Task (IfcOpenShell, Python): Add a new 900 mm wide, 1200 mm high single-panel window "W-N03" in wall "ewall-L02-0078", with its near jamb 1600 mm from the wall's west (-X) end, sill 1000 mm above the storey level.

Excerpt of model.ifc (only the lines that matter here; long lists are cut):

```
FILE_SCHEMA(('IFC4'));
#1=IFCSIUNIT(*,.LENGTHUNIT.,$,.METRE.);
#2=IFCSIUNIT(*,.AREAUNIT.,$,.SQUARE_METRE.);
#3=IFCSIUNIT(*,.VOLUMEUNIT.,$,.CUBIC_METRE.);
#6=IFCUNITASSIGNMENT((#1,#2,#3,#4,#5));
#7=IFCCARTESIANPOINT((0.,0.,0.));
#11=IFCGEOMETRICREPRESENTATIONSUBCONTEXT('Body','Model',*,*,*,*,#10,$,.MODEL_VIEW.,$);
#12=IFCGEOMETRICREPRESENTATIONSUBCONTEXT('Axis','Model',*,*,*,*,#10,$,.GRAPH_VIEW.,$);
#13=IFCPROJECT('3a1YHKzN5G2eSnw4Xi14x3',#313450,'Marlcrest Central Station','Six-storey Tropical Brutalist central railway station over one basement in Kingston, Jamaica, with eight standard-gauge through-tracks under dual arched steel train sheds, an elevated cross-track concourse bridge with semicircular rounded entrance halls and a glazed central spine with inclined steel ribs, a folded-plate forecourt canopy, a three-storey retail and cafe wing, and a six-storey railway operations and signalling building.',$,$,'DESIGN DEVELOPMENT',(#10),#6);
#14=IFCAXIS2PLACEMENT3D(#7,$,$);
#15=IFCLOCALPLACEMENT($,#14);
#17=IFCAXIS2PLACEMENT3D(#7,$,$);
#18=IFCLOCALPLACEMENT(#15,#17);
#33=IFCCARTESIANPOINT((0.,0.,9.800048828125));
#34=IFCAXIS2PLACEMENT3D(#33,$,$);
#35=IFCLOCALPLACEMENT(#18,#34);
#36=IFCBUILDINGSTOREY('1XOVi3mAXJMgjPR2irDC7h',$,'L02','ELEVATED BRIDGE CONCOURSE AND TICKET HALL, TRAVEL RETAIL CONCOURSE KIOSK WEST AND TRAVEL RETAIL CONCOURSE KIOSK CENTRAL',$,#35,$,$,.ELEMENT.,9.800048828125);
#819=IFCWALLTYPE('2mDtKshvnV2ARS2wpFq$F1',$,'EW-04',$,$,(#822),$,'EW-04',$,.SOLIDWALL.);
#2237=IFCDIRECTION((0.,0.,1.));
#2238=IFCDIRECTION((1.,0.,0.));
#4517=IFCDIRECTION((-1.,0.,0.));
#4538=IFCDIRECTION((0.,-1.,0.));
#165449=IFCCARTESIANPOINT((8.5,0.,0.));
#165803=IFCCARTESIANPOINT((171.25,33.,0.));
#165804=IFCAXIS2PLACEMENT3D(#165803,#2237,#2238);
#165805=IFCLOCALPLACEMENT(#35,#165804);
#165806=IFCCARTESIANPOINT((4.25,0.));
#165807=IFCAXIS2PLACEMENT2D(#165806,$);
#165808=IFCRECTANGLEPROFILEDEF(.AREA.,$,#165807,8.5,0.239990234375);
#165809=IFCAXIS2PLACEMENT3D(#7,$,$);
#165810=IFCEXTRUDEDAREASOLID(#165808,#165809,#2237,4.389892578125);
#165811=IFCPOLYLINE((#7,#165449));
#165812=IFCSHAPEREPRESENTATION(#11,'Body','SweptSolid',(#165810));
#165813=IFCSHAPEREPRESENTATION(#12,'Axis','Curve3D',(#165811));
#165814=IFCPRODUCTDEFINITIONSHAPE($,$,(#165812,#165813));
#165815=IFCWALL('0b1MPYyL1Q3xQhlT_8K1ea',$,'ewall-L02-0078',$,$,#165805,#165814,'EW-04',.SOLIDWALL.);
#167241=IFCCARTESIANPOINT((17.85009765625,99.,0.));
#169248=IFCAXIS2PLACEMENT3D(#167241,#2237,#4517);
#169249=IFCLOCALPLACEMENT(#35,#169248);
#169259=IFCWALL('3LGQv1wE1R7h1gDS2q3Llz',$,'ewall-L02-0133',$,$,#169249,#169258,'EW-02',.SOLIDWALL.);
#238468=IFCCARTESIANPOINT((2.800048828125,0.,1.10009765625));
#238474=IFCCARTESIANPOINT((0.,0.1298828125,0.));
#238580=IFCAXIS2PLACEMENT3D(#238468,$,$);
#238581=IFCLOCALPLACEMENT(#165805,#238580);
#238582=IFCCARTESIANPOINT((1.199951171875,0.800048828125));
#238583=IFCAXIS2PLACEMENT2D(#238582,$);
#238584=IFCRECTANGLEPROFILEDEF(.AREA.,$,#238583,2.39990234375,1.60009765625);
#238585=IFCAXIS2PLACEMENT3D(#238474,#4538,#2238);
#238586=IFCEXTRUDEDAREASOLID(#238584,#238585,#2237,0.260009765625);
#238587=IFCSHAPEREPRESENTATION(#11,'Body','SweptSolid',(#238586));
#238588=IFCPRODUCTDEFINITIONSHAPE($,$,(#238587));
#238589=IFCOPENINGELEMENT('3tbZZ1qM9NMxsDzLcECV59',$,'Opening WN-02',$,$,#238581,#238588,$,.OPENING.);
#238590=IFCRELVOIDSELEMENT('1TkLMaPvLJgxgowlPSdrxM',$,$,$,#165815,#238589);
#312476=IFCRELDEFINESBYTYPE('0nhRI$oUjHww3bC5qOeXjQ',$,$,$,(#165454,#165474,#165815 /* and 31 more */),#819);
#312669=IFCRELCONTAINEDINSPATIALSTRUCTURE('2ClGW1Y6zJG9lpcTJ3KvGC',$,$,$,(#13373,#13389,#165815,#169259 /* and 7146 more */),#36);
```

```python
import numpy as np
import ifcopenshell
import ifcopenshell.api.feature
import ifcopenshell.api.geometry
import ifcopenshell.api.root
import ifcopenshell.api.spatial
import ifcopenshell.geom
import ifcopenshell.util.element
import ifcopenshell.util.placement
import ifcopenshell.util.representation
import ifcopenshell.util.shape
import ifcopenshell.util.unit

model = ifcopenshell.open("model.ifc")
unit_scale = ifcopenshell.util.unit.calculate_unit_scale(model)
settings = ifcopenshell.geom.settings()


def volume(element):
    """Net volume in cubic metres, openings subtracted."""
    shape = ifcopenshell.geom.create_shape(settings, element)
    return ifcopenshell.util.shape.get_volume(shape.geometry)


wall = model.by_guid("0b1MPYyL1Q3xQhlT_8K1ea")
storey = ifcopenshell.util.element.get_container(wall, ifc_class="IfcBuildingStorey")
context = ifcopenshell.util.representation.get_context(model, "Model", "Body", "MODEL_VIEW")
before = volume(wall)

width, height, from_end, sill = 0.9, 1.2, 1.6, 1  # metres

# The wall runs along its own X axis, and the end named is its -X end.
wall_shape = ifcopenshell.geom.create_shape(settings, wall)
x, y, z = ifcopenshell.util.shape.get_vertices(wall_shape.geometry).T
start = x.min() + from_end
face, thickness = float(y.min()), float(y.max() - y.min())
wall_matrix = ifcopenshell.util.placement.get_local_placement(wall.ObjectPlacement)
level = ifcopenshell.util.placement.get_local_placement(storey.ObjectPlacement)[2, 3]


def in_wall(x, y):
    """Placement at x, y metres in the wall's axes, at sill height."""
    matrix = wall_matrix.copy()
    matrix[:, 3] = wall_matrix @ np.array([x / unit_scale, y / unit_scale, 0.0, 1.0])
    matrix[2, 3] = level + sill / unit_scale
    return matrix


# Opening: a box that overshoots both wall faces by 50 mm.
opening = ifcopenshell.api.root.create_entity(model, ifc_class="IfcOpeningElement", predefined_type="OPENING")
box = ifcopenshell.api.geometry.add_wall_representation(
    model, context=context, length=width, height=height, thickness=thickness + 0.1
)
ifcopenshell.api.geometry.assign_representation(model, product=opening, representation=box)
ifcopenshell.api.geometry.edit_object_placement(model, product=opening, matrix=in_wall(start, face - 0.05), is_si=False)
ifcopenshell.api.feature.add_feature(model, feature=opening, element=wall)

window = ifcopenshell.api.root.create_entity(model, ifc_class="IfcWindow", name="W-N03", predefined_type="WINDOW")
window.OverallWidth, window.OverallHeight = width / unit_scale, height / unit_scale
window.PartitioningType = "SINGLE_PANEL"
body = ifcopenshell.api.geometry.add_window_representation(
    model,
    context=context,
    overall_width=window.OverallWidth,
    overall_height=window.OverallHeight,
    partition_type="SINGLE_PANEL",
)
ifcopenshell.api.geometry.assign_representation(model, product=window, representation=body)
ifcopenshell.api.spatial.assign_container(model, products=[window], relating_structure=storey)
ifcopenshell.api.feature.add_filling(model, opening=opening, element=window)

# Centre the window in the wall's thickness.
ifcopenshell.api.geometry.edit_object_placement(model, product=window, matrix=in_wall(start, face), is_si=False)
window_shape = ifcopenshell.geom.create_shape(settings, window)
depth = ifcopenshell.util.shape.get_vertices(window_shape.geometry)[:, 1]
offset = face + thickness / 2 - (depth.min() + depth.max()) / 2
ifcopenshell.api.geometry.edit_object_placement(model, product=window, matrix=in_wall(start, offset), is_si=False)

after = volume(wall)

print(f"wall volume {before:.3f} -> {after:.3f} m3")

model.write("model_v2.ifc")
```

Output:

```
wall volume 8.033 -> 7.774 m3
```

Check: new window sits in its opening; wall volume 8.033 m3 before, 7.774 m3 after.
